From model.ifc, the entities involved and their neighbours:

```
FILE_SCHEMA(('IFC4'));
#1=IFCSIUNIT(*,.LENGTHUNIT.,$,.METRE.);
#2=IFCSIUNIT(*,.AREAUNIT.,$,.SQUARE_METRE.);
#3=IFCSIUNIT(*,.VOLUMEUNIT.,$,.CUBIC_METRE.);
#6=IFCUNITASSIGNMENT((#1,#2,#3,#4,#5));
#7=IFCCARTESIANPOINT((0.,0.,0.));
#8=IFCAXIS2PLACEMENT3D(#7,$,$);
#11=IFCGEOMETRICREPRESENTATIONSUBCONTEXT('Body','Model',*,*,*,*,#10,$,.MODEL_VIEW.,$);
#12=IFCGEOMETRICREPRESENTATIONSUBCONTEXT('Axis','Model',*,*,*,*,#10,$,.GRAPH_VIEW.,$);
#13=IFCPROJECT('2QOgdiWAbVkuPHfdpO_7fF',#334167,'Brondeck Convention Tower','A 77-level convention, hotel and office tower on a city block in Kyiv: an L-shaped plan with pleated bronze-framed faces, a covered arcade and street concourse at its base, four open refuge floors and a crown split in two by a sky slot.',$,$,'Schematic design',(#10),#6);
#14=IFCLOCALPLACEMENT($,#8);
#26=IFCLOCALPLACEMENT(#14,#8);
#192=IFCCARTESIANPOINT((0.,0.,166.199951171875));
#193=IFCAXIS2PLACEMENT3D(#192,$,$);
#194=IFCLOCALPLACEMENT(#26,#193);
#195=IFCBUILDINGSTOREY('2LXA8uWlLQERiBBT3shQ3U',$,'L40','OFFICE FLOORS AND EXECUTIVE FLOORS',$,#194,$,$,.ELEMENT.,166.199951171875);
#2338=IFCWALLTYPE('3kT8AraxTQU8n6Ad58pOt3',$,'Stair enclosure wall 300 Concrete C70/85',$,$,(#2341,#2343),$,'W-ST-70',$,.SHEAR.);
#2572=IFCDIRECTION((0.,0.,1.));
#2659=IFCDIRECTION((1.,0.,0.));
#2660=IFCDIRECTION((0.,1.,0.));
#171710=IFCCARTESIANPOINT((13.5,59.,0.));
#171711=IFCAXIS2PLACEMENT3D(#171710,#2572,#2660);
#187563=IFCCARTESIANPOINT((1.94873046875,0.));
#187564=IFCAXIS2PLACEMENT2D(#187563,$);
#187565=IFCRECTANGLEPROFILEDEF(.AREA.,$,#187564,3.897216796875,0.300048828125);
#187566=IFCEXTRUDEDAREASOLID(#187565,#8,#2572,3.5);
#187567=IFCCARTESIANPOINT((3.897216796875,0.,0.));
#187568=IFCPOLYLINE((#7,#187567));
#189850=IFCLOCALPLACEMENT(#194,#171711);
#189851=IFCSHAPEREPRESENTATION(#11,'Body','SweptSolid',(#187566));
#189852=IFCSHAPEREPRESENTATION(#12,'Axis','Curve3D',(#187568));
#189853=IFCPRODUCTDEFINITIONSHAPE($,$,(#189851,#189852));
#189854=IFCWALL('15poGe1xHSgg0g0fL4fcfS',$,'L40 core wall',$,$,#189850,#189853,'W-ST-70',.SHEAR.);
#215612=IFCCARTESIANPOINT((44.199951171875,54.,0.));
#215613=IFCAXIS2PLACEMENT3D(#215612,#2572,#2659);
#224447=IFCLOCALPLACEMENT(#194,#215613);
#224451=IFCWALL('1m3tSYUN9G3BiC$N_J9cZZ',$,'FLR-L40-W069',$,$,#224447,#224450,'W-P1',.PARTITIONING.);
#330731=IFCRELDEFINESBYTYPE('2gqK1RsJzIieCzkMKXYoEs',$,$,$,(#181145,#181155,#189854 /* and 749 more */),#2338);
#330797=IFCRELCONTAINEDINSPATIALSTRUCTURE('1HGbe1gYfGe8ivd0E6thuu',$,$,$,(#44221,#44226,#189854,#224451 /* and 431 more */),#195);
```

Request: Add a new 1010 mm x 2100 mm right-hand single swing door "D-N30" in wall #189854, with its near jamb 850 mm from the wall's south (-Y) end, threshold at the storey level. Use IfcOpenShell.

```python
import numpy as np
import ifcopenshell
import ifcopenshell.api.feature
import ifcopenshell.api.geometry
import ifcopenshell.api.root
import ifcopenshell.api.spatial
import ifcopenshell.geom
import ifcopenshell.util.element
import ifcopenshell.util.placement
import ifcopenshell.util.representation
import ifcopenshell.util.shape
import ifcopenshell.util.unit

model = ifcopenshell.open("model.ifc")
unit_scale = ifcopenshell.util.unit.calculate_unit_scale(model)
settings = ifcopenshell.geom.settings()


def volume(element):
    """Net volume in cubic metres, openings subtracted."""
    shape = ifcopenshell.geom.create_shape(settings, element)
    return ifcopenshell.util.shape.get_volume(shape.geometry)


wall = model.by_guid("15poGe1xHSgg0g0fL4fcfS")
storey = ifcopenshell.util.element.get_container(wall, ifc_class="IfcBuildingStorey")
context = ifcopenshell.util.representation.get_context(model, "Model", "Body", "MODEL_VIEW")
before = volume(wall)

width, height, from_end, sill = 1.01, 2.1, 0.85, 0.0  # metres

# The wall runs along its own X axis, and the end named is its -X end.
wall_shape = ifcopenshell.geom.create_shape(settings, wall)
x, y, z = ifcopenshell.util.shape.get_vertices(wall_shape.geometry).T
start = x.min() + from_end
face, thickness = float(y.min()), float(y.max() - y.min())
wall_matrix = ifcopenshell.util.placement.get_local_placement(wall.ObjectPlacement)
level = ifcopenshell.util.placement.get_local_placement(storey.ObjectPlacement)[2, 3]


def in_wall(x, y):
    """Placement at x, y metres in the wall's axes, at sill height."""
    matrix = wall_matrix.copy()
    matrix[:, 3] = wall_matrix @ np.array([x / unit_scale, y / unit_scale, 0.0, 1.0])
    matrix[2, 3] = level + sill / unit_scale
    return matrix


# Opening: a box that overshoots both wall faces by 50 mm.
opening = ifcopenshell.api.root.create_entity(model, ifc_class="IfcOpeningElement", predefined_type="OPENING")
box = ifcopenshell.api.geometry.add_wall_representation(
    model, context=context, length=width, height=height, thickness=thickness + 0.1
)
ifcopenshell.api.geometry.assign_representation(model, product=opening, representation=box)
ifcopenshell.api.geometry.edit_object_placement(model, product=opening, matrix=in_wall(start, face - 0.05), is_si=False)
ifcopenshell.api.feature.add_feature(model, feature=opening, element=wall)

door = ifcopenshell.api.root.create_entity(model, ifc_class="IfcDoor", name="D-N30", predefined_type="DOOR")
door.OverallWidth, door.OverallHeight = width / unit_scale, height / unit_scale
door.OperationType = "SINGLE_SWING_RIGHT"
body = ifcopenshell.api.geometry.add_door_representation(
    model,
    context=context,
    overall_width=door.OverallWidth,
    overall_height=door.OverallHeight,
    operation_type="SINGLE_SWING_RIGHT",
    lining_properties={"LiningDepth": thickness / unit_scale, "ThresholdDepth": thickness / unit_scale},
)
ifcopenshell.api.geometry.assign_representation(model, product=door, representation=body)
ifcopenshell.api.spatial.assign_container(model, products=[door], relating_structure=storey)
ifcopenshell.api.feature.add_filling(model, opening=opening, element=door)

# The lining spans the wall, so the door starts at the wall face.
ifcopenshell.api.geometry.edit_object_placement(model, product=door, matrix=in_wall(start, face), is_si=False)

after = volume(wall)

print(f"wall volume {before:.3f} -> {after:.3f} m3")

model.write("model_edited.ifc")
```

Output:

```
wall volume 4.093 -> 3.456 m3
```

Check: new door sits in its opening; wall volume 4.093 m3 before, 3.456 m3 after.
